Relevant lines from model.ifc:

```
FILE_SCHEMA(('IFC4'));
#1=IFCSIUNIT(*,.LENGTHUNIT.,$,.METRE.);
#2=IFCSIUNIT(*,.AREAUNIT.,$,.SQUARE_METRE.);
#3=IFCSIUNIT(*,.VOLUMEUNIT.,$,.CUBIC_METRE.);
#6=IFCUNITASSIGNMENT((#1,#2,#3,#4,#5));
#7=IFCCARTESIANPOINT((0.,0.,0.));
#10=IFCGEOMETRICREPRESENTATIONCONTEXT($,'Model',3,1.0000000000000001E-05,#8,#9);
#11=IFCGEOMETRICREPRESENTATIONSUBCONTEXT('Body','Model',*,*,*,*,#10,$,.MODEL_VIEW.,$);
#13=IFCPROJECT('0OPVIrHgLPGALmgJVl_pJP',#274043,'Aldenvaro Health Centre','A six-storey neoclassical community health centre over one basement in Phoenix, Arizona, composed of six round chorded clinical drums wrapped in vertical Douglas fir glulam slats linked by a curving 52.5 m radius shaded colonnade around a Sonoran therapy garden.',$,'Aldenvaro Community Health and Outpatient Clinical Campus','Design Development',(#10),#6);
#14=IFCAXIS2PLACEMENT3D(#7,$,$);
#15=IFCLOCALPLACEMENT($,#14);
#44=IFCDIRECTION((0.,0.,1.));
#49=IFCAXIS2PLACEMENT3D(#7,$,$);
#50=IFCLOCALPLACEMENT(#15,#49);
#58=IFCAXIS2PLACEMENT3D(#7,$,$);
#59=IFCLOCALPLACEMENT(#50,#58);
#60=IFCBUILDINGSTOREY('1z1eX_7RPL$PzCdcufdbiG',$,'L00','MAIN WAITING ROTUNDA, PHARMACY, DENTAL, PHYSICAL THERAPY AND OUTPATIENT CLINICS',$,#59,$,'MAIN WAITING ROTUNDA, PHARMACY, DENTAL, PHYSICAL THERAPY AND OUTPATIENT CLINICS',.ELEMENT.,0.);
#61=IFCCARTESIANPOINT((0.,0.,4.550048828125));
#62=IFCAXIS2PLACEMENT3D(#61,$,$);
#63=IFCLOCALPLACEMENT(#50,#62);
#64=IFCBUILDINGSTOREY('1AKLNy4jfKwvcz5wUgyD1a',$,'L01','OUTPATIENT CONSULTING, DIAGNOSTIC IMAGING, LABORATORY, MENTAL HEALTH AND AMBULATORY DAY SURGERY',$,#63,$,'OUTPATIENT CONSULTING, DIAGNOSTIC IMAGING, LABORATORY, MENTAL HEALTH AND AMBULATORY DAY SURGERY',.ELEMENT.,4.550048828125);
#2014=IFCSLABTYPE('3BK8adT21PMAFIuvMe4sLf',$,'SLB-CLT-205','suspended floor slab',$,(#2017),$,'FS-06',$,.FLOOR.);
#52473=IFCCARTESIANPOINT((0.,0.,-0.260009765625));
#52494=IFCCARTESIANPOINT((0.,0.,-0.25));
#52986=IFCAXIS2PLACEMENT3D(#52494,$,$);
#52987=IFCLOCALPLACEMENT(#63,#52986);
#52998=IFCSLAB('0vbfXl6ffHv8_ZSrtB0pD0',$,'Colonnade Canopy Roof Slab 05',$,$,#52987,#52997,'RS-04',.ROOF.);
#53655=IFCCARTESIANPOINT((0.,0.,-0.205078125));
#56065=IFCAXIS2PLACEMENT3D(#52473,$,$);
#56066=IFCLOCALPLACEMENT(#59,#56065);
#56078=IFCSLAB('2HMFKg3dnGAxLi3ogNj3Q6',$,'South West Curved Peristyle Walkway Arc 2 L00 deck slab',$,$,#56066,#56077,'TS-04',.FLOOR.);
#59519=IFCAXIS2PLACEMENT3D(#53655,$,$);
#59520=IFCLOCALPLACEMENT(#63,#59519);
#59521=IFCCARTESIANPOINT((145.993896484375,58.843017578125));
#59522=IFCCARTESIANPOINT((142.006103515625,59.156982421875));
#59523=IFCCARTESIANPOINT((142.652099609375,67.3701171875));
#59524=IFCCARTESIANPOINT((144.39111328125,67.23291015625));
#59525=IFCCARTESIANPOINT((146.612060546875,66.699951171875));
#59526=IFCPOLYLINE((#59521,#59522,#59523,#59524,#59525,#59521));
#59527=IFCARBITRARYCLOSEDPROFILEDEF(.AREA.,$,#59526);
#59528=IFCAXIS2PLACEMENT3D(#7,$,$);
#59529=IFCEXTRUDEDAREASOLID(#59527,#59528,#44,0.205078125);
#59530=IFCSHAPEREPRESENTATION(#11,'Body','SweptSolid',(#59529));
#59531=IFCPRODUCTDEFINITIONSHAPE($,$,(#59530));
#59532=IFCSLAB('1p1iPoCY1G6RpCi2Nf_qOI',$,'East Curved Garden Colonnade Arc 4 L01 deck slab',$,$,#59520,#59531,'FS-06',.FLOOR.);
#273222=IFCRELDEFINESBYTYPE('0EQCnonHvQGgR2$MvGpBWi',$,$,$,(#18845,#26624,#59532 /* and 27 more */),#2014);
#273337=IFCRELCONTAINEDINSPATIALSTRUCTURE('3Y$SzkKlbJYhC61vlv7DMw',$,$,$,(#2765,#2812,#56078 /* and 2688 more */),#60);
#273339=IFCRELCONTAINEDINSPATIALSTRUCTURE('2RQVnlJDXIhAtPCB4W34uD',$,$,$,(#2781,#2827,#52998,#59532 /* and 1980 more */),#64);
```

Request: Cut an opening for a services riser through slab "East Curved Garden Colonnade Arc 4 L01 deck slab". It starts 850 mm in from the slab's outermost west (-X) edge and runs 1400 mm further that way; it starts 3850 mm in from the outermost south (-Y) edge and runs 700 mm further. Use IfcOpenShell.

```python
import numpy as np
import ifcopenshell
import ifcopenshell.api.feature
import ifcopenshell.api.geometry
import ifcopenshell.api.root
import ifcopenshell.geom
import ifcopenshell.util.placement
import ifcopenshell.util.representation
import ifcopenshell.util.shape
import ifcopenshell.util.unit

model = ifcopenshell.open("model.ifc")
unit_scale = ifcopenshell.util.unit.calculate_unit_scale(model)
settings = ifcopenshell.geom.settings()


def volume(element):
    """Net volume in cubic metres, openings subtracted."""
    shape = ifcopenshell.geom.create_shape(settings, element)
    return ifcopenshell.util.shape.get_volume(shape.geometry)


slab = model.by_guid("1p1iPoCY1G6RpCi2Nf_qOI")
before = volume(slab)

# Extent in the slab's own axes, in metres. The edges named are its -X and -Y sides.
slab_shape = ifcopenshell.geom.create_shape(settings, slab)
vertices = ifcopenshell.util.shape.get_vertices(slab_shape.geometry)
x_min, y_min, bottom = vertices.min(axis=0)
top = vertices[:, 2].max()

opening = ifcopenshell.api.root.create_entity(model, ifc_class="IfcOpeningElement", name="Services riser opening", predefined_type="OPENING")
context = ifcopenshell.util.representation.get_context(model, "Model", "Body", "MODEL_VIEW")
width, depth = 1.4, 0.7
outline = [(0.0, 0.0), (width, 0.0), (width, depth), (0.0, depth), (0.0, 0.0)]
# Overshoot both faces by 50 mm so the cut is clean.
shape = ifcopenshell.api.geometry.add_slab_representation(
    model, context=context, depth=top - bottom + 0.1, polyline=outline
)
ifcopenshell.api.geometry.assign_representation(model, product=opening, representation=shape)

matrix = ifcopenshell.util.placement.get_local_placement(slab.ObjectPlacement)
matrix[:, 3] = matrix @ np.append(np.array([x_min + 0.85, y_min + 3.85, bottom - 0.05]) / unit_scale, 1.0)
ifcopenshell.api.geometry.edit_object_placement(model, product=opening, matrix=matrix, is_si=False)
ifcopenshell.api.feature.add_feature(model, feature=opening, element=slab)

after = volume(slab)

print(f"slab volume {before:.3f} -> {after:.3f} m3")

model.write("model_v2.ifc")
```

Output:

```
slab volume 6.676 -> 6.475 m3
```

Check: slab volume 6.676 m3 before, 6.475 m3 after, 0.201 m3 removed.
